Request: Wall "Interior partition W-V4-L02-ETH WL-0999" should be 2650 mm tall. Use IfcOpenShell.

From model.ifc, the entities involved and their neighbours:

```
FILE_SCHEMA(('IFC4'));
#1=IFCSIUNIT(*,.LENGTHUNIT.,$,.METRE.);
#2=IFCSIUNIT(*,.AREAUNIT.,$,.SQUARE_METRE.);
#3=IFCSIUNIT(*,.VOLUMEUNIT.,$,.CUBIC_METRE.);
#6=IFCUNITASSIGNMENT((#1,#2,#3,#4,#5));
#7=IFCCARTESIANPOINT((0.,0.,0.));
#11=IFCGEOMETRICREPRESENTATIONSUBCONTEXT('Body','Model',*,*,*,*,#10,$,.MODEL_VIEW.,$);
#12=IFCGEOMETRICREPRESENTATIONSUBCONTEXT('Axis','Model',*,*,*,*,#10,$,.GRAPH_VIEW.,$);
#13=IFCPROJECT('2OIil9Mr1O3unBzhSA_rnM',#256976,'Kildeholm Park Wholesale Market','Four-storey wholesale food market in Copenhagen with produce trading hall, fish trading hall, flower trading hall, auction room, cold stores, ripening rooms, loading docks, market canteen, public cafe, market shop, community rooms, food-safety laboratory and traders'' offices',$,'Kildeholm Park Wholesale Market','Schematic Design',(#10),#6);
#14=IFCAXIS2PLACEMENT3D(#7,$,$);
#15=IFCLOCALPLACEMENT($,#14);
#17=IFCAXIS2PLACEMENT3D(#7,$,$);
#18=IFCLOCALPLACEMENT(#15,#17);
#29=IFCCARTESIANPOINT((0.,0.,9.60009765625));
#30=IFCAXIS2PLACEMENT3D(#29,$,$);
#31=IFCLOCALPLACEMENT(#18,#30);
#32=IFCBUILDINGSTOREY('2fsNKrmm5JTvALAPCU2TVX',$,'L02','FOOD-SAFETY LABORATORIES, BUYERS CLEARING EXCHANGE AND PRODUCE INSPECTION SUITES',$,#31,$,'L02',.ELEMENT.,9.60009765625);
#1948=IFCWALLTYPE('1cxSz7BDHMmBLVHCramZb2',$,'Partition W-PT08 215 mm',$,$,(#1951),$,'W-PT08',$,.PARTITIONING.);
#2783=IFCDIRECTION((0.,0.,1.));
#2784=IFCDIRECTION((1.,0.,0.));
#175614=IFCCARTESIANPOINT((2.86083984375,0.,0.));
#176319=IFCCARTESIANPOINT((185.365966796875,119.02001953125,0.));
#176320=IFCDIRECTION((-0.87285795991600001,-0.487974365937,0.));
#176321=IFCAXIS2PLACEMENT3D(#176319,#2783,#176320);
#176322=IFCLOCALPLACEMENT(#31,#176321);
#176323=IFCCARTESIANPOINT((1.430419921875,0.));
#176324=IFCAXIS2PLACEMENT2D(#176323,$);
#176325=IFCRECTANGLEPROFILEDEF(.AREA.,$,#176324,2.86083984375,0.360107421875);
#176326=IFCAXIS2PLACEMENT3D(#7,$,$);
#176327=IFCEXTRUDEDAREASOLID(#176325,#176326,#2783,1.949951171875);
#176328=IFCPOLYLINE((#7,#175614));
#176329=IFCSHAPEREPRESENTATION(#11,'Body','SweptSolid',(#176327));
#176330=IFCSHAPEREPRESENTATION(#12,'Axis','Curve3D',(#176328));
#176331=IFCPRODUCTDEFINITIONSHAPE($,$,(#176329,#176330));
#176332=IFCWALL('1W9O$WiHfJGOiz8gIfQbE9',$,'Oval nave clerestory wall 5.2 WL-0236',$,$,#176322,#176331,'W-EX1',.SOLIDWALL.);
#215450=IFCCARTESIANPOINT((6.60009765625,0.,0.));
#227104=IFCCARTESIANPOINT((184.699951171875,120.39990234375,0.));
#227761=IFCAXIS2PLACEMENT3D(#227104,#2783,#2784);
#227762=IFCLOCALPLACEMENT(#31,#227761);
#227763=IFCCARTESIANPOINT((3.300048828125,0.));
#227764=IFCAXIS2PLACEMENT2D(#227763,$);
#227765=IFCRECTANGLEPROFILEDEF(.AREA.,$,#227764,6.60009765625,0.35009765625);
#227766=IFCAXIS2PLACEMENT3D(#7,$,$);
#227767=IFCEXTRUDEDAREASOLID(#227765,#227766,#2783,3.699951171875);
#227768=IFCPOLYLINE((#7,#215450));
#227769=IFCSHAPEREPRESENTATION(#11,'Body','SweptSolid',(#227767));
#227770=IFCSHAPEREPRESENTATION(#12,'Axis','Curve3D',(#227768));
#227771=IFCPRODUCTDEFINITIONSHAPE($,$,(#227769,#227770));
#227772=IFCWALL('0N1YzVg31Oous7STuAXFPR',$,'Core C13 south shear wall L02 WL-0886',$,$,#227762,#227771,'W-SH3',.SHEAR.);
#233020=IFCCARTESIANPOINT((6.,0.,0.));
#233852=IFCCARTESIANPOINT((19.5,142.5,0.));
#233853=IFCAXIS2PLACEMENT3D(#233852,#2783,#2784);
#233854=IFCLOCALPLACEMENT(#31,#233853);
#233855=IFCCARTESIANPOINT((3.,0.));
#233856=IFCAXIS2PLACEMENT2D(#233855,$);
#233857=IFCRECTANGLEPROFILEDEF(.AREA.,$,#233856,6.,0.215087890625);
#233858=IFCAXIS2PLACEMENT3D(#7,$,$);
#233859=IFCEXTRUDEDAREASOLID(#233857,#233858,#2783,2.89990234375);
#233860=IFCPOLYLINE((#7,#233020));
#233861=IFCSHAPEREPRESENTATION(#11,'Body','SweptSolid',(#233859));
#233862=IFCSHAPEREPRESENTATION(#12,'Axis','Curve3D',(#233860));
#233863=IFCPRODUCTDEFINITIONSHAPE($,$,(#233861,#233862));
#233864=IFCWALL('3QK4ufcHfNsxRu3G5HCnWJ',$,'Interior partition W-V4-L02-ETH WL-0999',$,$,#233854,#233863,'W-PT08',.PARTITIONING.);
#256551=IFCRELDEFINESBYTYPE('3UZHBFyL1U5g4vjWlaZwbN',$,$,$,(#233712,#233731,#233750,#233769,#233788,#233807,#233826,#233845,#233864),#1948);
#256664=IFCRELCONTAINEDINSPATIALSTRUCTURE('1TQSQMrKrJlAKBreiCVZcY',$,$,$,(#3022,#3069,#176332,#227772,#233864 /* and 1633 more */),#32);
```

```python
import ifcopenshell
import ifcopenshell.geom
import ifcopenshell.util.representation
import ifcopenshell.util.shape
import ifcopenshell.util.unit

model = ifcopenshell.open("model.ifc")
unit_scale = ifcopenshell.util.unit.calculate_unit_scale(model)
settings = ifcopenshell.geom.settings()


def volume(element):
    """Net volume in cubic metres, openings subtracted."""
    shape = ifcopenshell.geom.create_shape(settings, element)
    return ifcopenshell.util.shape.get_volume(shape.geometry)


wall = model.by_guid("3QK4ufcHfNsxRu3G5HCnWJ")
before = volume(wall)

body = ifcopenshell.util.representation.get_representation(wall, "Model", "Body")
solid = body.Items[0]
old_height = solid.Depth
solid.Depth = 2.65 / unit_scale
after = volume(wall)

print(f"height {old_height:g} -> {solid.Depth:g}, volume {before:.3f} -> {after:.3f} m3")

model.write("model-out.ifc")
```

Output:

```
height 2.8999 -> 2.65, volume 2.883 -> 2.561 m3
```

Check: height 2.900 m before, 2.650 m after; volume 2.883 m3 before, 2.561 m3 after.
